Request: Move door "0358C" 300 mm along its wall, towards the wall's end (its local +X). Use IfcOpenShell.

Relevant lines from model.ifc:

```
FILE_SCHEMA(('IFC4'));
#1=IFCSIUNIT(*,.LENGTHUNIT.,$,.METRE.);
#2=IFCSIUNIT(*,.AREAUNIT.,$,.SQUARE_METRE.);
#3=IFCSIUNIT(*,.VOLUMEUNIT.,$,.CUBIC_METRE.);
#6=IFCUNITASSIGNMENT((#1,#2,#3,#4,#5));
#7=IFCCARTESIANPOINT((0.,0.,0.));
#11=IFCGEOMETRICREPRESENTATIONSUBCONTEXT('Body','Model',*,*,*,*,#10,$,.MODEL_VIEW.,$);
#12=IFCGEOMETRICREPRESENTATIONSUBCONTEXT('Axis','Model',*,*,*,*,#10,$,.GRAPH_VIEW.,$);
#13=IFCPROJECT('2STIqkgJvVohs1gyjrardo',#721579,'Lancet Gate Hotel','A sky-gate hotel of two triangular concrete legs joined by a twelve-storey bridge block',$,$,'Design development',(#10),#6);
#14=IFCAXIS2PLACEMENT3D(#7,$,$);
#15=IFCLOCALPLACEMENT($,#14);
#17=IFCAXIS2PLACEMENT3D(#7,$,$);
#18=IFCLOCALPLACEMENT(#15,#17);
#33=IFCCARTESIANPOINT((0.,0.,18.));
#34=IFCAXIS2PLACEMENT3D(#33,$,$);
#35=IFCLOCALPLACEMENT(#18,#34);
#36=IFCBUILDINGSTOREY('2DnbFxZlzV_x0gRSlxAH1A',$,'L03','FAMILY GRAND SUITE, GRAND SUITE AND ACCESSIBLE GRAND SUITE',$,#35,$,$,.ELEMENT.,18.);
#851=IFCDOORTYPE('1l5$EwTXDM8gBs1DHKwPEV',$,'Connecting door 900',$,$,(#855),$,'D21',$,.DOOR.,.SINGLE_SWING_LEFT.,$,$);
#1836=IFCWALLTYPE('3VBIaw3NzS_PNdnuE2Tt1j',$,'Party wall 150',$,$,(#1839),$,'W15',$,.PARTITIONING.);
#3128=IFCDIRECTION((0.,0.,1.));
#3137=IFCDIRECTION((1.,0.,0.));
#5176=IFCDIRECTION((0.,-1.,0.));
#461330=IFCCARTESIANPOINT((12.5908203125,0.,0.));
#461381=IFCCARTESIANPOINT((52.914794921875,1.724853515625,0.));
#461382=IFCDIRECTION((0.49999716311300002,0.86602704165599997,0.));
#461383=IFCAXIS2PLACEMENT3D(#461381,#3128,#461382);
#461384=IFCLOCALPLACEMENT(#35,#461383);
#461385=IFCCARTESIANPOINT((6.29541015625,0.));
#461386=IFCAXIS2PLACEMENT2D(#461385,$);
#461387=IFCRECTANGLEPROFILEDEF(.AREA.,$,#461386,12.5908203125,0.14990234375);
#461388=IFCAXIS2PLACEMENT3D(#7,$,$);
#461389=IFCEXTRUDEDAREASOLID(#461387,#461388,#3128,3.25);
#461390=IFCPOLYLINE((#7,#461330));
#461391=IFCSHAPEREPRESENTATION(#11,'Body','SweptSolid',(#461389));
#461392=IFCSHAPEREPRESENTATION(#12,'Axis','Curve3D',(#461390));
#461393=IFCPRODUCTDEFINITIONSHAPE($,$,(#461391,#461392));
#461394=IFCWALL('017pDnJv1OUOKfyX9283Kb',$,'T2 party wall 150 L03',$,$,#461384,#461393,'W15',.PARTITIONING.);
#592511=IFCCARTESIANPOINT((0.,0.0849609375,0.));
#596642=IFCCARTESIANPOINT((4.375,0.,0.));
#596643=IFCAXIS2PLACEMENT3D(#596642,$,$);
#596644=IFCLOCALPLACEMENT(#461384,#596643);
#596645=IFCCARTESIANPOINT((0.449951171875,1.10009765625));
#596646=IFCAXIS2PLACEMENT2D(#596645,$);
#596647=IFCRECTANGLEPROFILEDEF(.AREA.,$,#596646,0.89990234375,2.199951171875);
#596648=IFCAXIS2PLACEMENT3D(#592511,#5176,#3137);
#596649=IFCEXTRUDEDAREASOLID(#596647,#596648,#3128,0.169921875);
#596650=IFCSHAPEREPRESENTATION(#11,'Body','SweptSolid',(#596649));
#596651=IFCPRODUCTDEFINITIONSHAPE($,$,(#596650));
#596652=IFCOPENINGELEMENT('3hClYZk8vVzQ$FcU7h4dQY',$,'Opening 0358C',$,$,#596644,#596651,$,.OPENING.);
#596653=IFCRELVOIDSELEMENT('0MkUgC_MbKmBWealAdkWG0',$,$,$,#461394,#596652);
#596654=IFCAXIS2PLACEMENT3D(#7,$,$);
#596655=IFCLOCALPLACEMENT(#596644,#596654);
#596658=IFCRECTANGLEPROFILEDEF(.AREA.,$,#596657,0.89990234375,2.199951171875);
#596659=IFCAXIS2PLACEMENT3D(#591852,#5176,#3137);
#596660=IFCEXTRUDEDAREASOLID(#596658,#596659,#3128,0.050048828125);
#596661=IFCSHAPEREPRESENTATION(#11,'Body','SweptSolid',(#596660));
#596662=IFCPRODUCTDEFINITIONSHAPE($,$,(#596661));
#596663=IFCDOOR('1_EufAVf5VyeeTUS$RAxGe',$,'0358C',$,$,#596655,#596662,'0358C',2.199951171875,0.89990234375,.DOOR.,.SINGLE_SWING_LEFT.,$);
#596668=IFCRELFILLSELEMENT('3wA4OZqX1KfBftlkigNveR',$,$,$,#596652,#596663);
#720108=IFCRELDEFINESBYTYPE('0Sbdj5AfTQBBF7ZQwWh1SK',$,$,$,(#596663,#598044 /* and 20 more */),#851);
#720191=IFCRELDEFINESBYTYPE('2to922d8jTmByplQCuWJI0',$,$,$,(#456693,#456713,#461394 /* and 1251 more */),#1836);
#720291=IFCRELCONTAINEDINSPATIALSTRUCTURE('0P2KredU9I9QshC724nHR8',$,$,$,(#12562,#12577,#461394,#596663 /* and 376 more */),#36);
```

```python
import ifcopenshell
import ifcopenshell.api.geometry
import ifcopenshell.util.placement
import ifcopenshell.util.unit

model = ifcopenshell.open("model.ifc")
unit_scale = ifcopenshell.util.unit.calculate_unit_scale(model)

door = model.by_guid("1_EufAVf5VyeeTUS$RAxGe")
opening = door.FillsVoids[0].RelatingOpeningElement
wall = opening.VoidsElements[0].RelatingBuildingElement

wall_matrix = ifcopenshell.util.placement.get_local_placement(wall.ObjectPlacement)
shift = wall_matrix[:3, 0] * 0.3 / unit_scale
before = ifcopenshell.util.placement.get_local_placement(door.ObjectPlacement)[:3, 3].copy()

# The door is placed relative to its opening, so it follows when the opening moves.
matrix = ifcopenshell.util.placement.get_local_placement(opening.ObjectPlacement)
matrix[:3, 3] += shift
ifcopenshell.api.geometry.edit_object_placement(
    model, product=opening, matrix=matrix, is_si=False, should_transform_children=True
)

after = ifcopenshell.util.placement.get_local_placement(door.ObjectPlacement)[:3, 3]
print("door moved by", (after - before).round(3) + 0.0)

model.write("model_updated.ifc")
```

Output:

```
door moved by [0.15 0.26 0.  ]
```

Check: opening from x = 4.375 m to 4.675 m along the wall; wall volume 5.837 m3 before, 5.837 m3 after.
